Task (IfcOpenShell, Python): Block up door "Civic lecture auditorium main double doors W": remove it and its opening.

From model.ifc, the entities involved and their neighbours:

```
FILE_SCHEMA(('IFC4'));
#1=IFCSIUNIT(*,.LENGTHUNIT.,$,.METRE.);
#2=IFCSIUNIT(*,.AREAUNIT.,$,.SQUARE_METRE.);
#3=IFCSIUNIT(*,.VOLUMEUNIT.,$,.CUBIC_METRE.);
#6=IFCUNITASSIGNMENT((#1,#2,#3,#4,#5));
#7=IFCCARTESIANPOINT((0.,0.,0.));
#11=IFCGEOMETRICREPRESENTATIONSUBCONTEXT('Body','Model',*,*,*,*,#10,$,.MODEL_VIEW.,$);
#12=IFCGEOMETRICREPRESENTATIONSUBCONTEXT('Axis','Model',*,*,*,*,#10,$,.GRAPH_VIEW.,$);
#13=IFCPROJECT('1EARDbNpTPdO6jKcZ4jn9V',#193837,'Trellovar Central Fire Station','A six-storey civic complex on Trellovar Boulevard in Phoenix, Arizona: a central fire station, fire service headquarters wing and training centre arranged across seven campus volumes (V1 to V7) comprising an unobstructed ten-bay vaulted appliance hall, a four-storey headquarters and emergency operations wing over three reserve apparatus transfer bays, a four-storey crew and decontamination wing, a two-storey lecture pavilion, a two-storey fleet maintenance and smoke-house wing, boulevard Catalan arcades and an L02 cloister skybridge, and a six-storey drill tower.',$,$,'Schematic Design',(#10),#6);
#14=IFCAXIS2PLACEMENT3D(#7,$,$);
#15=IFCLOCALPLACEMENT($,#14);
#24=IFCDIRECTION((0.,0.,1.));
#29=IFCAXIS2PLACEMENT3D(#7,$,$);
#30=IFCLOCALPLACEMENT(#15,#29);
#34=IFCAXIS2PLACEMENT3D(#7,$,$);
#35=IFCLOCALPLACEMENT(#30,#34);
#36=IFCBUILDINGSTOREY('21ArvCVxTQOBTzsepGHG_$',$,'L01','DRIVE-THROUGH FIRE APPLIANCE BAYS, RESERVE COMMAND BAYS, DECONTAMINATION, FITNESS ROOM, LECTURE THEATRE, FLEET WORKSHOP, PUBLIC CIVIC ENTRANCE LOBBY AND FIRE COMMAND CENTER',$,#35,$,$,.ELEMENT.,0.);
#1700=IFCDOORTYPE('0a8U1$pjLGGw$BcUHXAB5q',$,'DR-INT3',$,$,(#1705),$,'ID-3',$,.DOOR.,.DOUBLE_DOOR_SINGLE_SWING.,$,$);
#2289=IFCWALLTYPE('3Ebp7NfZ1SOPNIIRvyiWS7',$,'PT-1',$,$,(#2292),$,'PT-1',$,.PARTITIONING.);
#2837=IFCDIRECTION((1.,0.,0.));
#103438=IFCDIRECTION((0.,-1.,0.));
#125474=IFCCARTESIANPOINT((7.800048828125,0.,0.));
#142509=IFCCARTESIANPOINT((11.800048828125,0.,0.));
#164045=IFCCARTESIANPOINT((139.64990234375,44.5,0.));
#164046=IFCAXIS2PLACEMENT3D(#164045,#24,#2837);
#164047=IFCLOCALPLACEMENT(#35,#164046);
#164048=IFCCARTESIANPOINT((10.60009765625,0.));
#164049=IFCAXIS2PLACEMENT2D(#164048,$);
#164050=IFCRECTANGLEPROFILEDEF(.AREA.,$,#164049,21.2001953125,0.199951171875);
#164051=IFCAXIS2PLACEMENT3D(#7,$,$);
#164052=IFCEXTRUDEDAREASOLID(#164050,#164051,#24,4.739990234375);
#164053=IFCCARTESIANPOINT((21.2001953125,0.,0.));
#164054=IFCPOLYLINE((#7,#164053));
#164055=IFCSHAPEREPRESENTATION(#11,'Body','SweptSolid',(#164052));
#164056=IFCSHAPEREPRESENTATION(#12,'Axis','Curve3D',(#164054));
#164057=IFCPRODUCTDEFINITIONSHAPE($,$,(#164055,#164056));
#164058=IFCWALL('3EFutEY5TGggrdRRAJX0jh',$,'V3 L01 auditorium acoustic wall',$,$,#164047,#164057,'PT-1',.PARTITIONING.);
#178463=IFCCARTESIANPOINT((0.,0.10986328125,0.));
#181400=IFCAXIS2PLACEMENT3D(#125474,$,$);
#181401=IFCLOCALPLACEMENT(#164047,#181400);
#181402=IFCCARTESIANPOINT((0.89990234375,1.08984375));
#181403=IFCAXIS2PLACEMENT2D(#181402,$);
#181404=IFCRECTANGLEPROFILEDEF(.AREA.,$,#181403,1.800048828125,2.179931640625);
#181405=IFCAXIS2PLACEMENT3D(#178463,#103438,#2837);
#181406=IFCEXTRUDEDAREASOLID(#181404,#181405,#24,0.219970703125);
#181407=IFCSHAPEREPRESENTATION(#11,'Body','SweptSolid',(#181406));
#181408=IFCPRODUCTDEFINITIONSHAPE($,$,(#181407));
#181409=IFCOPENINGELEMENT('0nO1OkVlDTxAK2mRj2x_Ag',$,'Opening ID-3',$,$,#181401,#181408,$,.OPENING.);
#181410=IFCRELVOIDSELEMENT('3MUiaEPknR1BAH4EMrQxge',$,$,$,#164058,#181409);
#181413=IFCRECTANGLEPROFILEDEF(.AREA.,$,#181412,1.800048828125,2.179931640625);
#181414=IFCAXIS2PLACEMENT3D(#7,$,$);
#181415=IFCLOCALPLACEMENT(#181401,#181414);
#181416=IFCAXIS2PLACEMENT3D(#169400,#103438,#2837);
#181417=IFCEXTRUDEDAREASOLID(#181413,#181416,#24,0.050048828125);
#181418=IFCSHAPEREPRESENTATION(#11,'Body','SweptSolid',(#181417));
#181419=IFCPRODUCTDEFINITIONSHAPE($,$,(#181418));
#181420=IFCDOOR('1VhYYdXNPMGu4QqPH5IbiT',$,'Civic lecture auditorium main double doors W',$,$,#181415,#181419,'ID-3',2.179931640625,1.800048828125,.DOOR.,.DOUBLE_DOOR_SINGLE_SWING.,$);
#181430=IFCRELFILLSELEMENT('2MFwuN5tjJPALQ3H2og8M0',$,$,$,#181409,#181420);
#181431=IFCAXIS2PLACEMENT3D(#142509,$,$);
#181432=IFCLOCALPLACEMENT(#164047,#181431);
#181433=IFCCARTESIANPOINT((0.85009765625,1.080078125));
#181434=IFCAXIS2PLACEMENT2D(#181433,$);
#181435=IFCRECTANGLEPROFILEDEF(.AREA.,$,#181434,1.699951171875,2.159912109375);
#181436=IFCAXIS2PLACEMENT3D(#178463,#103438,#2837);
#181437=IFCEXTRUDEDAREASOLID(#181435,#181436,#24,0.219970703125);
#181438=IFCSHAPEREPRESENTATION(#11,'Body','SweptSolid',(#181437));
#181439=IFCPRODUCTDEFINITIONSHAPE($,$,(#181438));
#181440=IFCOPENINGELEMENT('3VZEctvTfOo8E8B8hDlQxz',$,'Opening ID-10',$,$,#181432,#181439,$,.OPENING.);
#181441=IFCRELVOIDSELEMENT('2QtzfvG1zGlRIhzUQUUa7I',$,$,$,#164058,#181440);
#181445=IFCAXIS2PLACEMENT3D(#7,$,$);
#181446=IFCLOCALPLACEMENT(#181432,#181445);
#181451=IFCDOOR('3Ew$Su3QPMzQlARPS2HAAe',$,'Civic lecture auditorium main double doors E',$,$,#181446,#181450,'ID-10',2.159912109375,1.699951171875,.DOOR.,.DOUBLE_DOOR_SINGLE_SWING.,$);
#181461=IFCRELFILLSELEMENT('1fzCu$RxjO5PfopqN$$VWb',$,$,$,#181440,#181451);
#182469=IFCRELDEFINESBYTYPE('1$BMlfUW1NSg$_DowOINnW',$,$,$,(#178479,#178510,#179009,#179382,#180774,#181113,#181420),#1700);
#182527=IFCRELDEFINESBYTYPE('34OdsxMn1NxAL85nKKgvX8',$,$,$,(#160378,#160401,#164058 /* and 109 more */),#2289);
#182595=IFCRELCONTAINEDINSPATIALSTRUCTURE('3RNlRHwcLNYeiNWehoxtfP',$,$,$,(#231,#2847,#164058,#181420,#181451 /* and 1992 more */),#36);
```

```python
import ifcopenshell
import ifcopenshell.api.feature
import ifcopenshell.api.root
import ifcopenshell.geom
import ifcopenshell.util.shape

model = ifcopenshell.open("model.ifc")
settings = ifcopenshell.geom.settings()


def volume(element):
    """Net volume in cubic metres, openings subtracted."""
    shape = ifcopenshell.geom.create_shape(settings, element)
    return ifcopenshell.util.shape.get_volume(shape.geometry)


door = model.by_guid("1VhYYdXNPMGu4QqPH5IbiT")
opening = door.FillsVoids[0].RelatingOpeningElement
wall = opening.VoidsElements[0].RelatingBuildingElement
before = volume(wall)

ifcopenshell.api.root.remove_product(model, product=door)
ifcopenshell.api.feature.remove_feature(model, feature=opening)

after = volume(wall)

print(f"wall volume {before:.3f} -> {after:.3f} m3")

model.write("model_updated.ifc")
```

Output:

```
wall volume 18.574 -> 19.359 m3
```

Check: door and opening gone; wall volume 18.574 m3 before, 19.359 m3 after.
